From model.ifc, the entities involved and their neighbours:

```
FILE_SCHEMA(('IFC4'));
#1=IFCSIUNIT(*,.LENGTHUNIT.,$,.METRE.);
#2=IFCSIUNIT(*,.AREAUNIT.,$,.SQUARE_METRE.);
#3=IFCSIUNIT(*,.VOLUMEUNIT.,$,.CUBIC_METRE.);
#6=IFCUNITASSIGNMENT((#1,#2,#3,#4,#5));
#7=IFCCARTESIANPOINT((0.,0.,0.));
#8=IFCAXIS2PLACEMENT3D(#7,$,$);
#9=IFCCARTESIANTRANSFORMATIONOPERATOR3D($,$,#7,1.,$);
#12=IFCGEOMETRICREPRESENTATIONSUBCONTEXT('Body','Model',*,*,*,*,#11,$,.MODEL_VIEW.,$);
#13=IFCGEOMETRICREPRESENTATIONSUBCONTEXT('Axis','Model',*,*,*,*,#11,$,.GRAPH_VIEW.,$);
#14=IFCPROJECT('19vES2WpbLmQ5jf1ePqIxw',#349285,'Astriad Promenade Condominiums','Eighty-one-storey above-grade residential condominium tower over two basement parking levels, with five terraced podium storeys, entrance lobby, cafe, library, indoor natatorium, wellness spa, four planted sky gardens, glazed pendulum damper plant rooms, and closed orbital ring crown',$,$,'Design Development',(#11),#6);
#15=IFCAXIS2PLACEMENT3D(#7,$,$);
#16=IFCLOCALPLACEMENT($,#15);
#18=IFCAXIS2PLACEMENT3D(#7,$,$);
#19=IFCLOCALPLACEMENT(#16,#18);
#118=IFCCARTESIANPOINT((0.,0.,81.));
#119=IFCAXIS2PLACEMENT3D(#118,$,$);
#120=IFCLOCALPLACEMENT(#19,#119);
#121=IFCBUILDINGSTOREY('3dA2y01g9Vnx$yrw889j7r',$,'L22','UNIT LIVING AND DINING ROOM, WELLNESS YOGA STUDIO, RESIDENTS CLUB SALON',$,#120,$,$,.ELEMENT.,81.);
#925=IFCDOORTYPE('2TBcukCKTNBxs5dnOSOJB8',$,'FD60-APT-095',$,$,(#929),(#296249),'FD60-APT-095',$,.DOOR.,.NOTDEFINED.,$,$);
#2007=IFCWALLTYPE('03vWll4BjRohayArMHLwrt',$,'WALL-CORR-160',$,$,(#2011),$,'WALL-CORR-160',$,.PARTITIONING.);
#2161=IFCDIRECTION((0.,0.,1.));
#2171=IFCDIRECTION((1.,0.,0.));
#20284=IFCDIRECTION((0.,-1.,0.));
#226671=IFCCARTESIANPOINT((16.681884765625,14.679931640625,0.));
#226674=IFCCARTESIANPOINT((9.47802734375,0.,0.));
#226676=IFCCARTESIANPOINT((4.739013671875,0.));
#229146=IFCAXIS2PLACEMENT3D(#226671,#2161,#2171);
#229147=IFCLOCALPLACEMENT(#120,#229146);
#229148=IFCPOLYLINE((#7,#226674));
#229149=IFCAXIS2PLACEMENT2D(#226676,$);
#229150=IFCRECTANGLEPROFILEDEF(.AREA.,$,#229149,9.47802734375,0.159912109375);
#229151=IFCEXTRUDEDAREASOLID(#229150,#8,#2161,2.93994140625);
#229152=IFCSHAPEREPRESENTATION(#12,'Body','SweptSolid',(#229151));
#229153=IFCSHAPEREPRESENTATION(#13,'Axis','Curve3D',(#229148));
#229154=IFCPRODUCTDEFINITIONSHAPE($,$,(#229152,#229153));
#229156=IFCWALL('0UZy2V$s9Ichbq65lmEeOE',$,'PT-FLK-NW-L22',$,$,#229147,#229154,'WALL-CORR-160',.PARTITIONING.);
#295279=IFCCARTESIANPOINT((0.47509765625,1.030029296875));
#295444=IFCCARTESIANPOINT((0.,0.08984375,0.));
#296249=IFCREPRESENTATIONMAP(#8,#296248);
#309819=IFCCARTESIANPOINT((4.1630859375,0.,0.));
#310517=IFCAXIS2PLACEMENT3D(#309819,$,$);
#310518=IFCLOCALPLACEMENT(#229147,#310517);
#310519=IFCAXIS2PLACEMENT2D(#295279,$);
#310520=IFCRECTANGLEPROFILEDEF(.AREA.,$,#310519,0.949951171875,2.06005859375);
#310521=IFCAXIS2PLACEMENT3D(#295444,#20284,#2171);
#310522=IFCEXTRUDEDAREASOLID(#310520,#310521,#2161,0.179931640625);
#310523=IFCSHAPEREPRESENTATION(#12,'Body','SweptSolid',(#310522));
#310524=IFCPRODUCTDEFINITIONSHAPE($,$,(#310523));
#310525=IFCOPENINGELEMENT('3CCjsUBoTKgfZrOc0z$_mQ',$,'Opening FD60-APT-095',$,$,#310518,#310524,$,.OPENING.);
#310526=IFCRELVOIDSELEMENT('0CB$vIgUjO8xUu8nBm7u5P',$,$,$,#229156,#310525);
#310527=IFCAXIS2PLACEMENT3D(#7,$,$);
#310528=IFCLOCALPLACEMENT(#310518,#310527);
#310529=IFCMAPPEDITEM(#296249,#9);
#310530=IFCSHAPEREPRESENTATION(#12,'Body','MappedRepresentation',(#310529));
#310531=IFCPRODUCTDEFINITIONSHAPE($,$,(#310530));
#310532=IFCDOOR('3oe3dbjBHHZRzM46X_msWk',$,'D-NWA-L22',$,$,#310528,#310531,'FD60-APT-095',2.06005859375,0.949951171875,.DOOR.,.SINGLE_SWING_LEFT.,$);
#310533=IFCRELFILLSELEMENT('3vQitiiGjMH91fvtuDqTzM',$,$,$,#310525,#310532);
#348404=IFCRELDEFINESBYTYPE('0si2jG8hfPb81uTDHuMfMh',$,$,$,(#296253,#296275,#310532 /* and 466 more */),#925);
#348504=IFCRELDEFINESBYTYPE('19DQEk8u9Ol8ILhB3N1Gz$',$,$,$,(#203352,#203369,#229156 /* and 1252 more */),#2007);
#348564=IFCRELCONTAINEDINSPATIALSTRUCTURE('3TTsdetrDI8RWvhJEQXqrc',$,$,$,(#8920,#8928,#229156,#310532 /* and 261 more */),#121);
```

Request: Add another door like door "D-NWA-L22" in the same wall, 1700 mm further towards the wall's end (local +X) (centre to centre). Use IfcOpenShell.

```python
import ifcopenshell
import ifcopenshell.api.feature
import ifcopenshell.api.geometry
import ifcopenshell.api.root
import ifcopenshell.geom
import ifcopenshell.util.element
import ifcopenshell.util.placement
import ifcopenshell.util.shape
import ifcopenshell.util.unit

model = ifcopenshell.open("model.ifc")
unit_scale = ifcopenshell.util.unit.calculate_unit_scale(model)
settings = ifcopenshell.geom.settings()


def volume(element):
    """Net volume in cubic metres, openings subtracted."""
    shape = ifcopenshell.geom.create_shape(settings, element)
    return ifcopenshell.util.shape.get_volume(shape.geometry)


door = model.by_guid("3oe3dbjBHHZRzM46X_msWk")
opening = door.FillsVoids[0].RelatingOpeningElement
wall = opening.VoidsElements[0].RelatingBuildingElement
before = volume(wall)
shift = ifcopenshell.util.placement.get_local_placement(wall.ObjectPlacement)[:3, 0] * 1.7 / unit_scale

# copy_class copies the void relationship, type, container and properties, but no geometry.
new_opening = ifcopenshell.api.root.copy_class(model, product=opening)
new_opening.Representation = ifcopenshell.util.element.copy_deep(
    model, opening.Representation, exclude=["IfcGeometricRepresentationContext", "IfcRepresentationMap"]
)
new_door = ifcopenshell.api.root.copy_class(model, product=door)
new_door.Representation = ifcopenshell.util.element.copy_deep(
    model, door.Representation, exclude=["IfcGeometricRepresentationContext", "IfcRepresentationMap"]
)
new_door.Tag = None
ifcopenshell.api.feature.add_filling(model, opening=new_opening, element=new_door)

for old, new in ((opening, new_opening), (door, new_door)):
    matrix = ifcopenshell.util.placement.get_local_placement(old.ObjectPlacement)
    matrix[:3, 3] += shift
    ifcopenshell.api.geometry.edit_object_placement(model, product=new, matrix=matrix, is_si=False)

after = volume(wall)

print(f"wall volume {before:.3f} -> {after:.3f} m3")

model.write("model_v2.ifc")
```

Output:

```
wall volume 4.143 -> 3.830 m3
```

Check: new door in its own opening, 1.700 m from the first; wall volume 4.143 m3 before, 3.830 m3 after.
